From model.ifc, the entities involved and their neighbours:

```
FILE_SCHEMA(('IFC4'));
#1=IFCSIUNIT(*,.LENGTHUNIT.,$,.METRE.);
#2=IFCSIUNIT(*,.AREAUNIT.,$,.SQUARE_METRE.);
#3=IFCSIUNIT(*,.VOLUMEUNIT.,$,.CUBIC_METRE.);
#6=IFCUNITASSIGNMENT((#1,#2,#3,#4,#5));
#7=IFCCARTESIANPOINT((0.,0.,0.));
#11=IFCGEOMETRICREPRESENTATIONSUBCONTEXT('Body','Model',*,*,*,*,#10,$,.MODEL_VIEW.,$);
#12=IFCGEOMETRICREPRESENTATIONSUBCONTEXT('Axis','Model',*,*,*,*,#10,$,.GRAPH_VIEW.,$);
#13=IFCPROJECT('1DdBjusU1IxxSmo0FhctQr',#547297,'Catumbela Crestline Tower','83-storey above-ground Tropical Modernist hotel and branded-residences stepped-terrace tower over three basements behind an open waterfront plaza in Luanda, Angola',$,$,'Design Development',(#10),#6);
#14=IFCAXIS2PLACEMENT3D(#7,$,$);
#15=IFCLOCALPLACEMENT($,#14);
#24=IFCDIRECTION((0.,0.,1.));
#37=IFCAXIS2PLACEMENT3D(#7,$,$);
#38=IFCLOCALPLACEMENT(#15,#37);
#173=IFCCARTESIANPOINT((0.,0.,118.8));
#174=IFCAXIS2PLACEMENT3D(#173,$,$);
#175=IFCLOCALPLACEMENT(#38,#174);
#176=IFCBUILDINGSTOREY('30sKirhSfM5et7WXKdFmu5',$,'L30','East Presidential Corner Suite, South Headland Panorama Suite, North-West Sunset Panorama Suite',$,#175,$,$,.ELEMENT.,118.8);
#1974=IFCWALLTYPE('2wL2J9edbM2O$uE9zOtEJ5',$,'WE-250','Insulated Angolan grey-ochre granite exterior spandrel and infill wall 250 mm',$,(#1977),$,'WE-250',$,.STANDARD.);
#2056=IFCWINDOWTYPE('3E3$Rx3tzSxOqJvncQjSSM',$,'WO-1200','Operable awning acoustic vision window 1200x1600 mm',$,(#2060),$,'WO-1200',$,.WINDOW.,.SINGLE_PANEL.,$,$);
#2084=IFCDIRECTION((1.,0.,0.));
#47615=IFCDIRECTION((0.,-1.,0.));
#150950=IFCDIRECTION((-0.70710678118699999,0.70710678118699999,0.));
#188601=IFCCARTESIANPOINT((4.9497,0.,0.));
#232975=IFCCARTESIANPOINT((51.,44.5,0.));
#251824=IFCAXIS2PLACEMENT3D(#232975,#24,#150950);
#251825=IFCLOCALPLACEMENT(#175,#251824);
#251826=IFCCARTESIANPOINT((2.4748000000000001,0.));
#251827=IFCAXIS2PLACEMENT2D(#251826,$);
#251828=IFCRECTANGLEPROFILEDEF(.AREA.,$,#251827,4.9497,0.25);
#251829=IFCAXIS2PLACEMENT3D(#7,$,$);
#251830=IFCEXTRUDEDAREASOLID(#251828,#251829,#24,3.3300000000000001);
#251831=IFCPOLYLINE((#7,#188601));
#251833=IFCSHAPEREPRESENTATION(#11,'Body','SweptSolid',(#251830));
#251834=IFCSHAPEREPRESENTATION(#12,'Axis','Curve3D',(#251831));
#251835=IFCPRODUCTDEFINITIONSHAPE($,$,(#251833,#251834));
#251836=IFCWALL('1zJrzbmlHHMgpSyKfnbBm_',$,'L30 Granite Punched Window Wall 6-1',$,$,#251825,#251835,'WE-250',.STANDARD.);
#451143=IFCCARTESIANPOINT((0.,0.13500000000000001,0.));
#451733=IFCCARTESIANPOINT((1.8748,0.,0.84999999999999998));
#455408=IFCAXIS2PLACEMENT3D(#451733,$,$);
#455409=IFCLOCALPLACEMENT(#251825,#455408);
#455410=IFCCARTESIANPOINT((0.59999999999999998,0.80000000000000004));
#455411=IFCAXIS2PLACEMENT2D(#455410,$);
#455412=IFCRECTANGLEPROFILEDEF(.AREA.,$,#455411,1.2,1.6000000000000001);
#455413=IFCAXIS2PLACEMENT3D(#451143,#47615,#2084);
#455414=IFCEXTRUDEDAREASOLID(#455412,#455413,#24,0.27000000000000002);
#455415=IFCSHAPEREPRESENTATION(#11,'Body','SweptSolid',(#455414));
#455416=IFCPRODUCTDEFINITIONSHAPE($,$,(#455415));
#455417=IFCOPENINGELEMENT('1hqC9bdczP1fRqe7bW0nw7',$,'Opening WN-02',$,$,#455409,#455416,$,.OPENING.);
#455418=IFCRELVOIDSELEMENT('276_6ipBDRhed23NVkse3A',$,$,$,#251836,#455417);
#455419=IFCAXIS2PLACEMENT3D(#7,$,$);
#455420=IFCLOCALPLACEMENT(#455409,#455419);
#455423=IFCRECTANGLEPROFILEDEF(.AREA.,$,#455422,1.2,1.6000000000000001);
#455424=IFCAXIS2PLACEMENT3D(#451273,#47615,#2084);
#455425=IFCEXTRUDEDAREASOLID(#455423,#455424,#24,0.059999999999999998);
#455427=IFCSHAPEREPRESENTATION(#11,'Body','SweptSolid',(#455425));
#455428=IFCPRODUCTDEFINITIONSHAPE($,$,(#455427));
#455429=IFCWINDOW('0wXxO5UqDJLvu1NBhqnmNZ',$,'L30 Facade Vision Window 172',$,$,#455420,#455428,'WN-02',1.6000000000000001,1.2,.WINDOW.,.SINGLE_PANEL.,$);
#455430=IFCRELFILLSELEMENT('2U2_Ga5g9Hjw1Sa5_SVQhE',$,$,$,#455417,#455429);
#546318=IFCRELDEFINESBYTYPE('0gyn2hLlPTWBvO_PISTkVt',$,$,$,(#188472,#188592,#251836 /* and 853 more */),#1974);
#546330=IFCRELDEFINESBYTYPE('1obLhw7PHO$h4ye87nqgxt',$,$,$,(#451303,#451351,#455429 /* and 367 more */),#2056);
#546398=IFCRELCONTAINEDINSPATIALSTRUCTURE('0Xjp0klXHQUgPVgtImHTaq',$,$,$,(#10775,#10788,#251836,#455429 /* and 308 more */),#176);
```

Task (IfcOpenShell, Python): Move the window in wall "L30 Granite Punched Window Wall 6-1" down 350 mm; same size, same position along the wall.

```python
import numpy as np
import ifcopenshell
import ifcopenshell.api.geometry
import ifcopenshell.util.placement
import ifcopenshell.util.unit

model = ifcopenshell.open("model.ifc")
unit_scale = ifcopenshell.util.unit.calculate_unit_scale(model)

window = model.by_id(455429)
opening = window.FillsVoids[0].RelatingOpeningElement
dz = -0.35 / unit_scale

shift = np.array([0.0, 0.0, dz])
# The window is placed relative to its opening, so it follows when the opening moves.
matrix = ifcopenshell.util.placement.get_local_placement(opening.ObjectPlacement)
matrix[:3, 3] += shift
ifcopenshell.api.geometry.edit_object_placement(
    model, product=opening, matrix=matrix, is_si=False, should_transform_children=True
)

print(f"moved by {dz * unit_scale:+.3f} m")

model.write("model-out.ifc")
```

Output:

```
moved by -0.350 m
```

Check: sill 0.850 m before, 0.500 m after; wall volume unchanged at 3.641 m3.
